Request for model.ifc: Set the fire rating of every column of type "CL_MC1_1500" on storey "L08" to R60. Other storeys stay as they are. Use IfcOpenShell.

First a look at what the model holds.

```python
import ifcopenshell
import ifcopenshell.util.element

model = ifcopenshell.open("model.ifc")
print(model.schema)
storey = next(s for s in model.by_type("IfcBuildingStorey") if s.Name == "L08")
columns = [e for e in ifcopenshell.util.element.get_decomposition(storey) if e.is_a("IfcColumn")]
seen = {}
for e in columns:
    element_type = ifcopenshell.util.element.get_type(e)
    key = (element_type.Name if element_type != e and element_type else None, ifcopenshell.util.element.get_pset(e, "Pset_ColumnCommon", "FireRating"))
    seen[key] = seen.get(key, 0) + 1
for (name, value), count in sorted(seen.items(), key=str):
    print(count, "x", name, "|", value)
```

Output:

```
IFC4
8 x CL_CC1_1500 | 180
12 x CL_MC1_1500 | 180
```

```python
import ifcopenshell
import ifcopenshell.api.pset
import ifcopenshell.util.element

model = ifcopenshell.open("model.ifc")

storey = next(s for s in model.by_type("IfcBuildingStorey") if s.Name == "L08")
columns = [e for e in ifcopenshell.util.element.get_decomposition(storey) if e.is_a("IfcColumn")]

count = 0
for e in columns:
    element_type = ifcopenshell.util.element.get_type(e)
    if element_type in (None, e) or element_type.Name != "CL_MC1_1500":
        continue
    found = ifcopenshell.util.element.get_pset(e, "Pset_ColumnCommon", should_inherit=False)
    if found:
        pset = model.by_id(found["id"])
        if len(ifcopenshell.util.element.get_elements_by_pset(pset)) > 1:
            pset = ifcopenshell.api.pset.unshare_pset(model, products=[e], pset=pset)[0]
    else:
        pset = ifcopenshell.api.pset.add_pset(model, product=e, name="Pset_ColumnCommon")
    ifcopenshell.api.pset.edit_pset(model, pset=pset, properties={"FireRating": "R60"})
    count += 1

print(count, "columns updated")

model.write("model_rev.ifc")
```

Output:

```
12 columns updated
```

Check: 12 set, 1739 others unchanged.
